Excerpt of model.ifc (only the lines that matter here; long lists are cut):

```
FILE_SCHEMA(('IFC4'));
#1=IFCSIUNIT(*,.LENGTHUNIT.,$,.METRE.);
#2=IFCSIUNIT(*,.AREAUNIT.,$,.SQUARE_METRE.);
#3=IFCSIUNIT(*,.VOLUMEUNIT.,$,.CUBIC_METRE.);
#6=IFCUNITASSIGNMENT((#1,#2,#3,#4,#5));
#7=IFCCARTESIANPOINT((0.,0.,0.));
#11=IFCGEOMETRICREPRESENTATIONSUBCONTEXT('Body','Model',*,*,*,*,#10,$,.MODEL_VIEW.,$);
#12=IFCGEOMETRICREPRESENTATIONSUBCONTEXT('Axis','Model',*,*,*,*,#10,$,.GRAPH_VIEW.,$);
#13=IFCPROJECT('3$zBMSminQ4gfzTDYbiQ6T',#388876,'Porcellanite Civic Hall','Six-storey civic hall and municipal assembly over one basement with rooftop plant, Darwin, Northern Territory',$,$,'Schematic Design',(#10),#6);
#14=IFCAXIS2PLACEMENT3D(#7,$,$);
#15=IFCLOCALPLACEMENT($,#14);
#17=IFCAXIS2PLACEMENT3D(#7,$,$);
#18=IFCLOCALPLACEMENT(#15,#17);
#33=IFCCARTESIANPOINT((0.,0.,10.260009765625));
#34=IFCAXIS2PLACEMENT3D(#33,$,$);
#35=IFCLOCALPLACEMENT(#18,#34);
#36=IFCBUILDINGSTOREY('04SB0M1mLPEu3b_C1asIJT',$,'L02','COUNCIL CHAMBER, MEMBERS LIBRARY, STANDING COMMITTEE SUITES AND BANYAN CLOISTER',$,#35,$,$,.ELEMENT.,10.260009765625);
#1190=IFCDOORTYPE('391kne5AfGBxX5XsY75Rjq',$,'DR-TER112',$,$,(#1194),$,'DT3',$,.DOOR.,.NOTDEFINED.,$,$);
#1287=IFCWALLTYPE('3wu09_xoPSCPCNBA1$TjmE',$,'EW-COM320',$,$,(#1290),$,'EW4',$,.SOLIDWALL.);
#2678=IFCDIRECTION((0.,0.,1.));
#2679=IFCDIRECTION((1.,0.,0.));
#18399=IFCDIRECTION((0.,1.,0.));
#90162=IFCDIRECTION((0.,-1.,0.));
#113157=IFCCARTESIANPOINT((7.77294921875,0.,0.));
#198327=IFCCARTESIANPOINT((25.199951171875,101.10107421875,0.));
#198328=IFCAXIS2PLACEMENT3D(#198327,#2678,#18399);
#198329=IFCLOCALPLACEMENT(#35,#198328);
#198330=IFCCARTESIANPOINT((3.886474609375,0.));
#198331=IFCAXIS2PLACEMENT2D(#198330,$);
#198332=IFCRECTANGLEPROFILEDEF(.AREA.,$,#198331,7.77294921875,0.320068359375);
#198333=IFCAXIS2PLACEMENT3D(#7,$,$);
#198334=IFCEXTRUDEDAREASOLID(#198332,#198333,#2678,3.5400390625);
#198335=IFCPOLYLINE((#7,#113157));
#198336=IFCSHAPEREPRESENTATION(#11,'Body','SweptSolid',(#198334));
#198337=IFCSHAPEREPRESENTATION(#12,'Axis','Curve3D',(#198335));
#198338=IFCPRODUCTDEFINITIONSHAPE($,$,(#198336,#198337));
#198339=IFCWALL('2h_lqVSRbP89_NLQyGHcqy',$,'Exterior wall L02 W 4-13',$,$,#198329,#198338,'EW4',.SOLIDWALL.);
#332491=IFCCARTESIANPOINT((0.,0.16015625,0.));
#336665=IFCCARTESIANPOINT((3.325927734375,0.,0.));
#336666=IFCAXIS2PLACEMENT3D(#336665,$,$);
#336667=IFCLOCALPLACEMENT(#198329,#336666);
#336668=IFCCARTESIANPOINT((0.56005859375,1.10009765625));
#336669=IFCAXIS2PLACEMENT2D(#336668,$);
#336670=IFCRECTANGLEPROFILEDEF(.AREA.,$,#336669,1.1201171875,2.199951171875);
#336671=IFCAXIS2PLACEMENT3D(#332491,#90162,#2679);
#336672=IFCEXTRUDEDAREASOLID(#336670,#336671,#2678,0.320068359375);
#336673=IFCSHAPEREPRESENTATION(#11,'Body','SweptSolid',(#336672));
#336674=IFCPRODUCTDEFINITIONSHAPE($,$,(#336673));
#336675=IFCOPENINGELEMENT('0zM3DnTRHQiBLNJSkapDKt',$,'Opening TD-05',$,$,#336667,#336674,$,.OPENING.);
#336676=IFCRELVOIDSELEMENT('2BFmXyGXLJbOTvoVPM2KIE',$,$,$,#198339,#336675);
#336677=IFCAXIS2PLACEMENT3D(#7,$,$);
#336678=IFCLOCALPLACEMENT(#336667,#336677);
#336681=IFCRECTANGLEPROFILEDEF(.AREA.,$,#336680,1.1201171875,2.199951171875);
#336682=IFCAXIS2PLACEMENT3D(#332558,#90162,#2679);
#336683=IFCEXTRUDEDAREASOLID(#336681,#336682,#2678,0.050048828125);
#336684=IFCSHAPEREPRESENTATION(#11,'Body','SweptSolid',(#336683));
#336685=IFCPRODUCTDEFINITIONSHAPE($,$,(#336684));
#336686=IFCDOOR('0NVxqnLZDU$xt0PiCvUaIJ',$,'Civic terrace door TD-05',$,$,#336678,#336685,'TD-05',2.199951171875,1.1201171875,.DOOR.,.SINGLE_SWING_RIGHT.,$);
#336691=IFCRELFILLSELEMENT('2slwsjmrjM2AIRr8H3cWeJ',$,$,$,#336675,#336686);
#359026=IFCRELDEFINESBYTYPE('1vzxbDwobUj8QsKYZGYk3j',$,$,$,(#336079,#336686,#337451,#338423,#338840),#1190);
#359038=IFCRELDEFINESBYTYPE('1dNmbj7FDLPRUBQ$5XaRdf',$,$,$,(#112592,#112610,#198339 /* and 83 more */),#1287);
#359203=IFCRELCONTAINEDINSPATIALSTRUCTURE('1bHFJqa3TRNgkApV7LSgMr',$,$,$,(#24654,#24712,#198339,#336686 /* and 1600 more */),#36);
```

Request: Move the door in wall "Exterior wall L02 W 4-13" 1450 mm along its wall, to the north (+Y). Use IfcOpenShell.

```python
import ifcopenshell
import ifcopenshell.api.geometry
import ifcopenshell.util.placement
import ifcopenshell.util.unit

model = ifcopenshell.open("model.ifc")
unit_scale = ifcopenshell.util.unit.calculate_unit_scale(model)

door = model.by_id(336686)
opening = door.FillsVoids[0].RelatingOpeningElement
wall = opening.VoidsElements[0].RelatingBuildingElement

wall_matrix = ifcopenshell.util.placement.get_local_placement(wall.ObjectPlacement)
shift = wall_matrix[:3, 0] * 1.45 / unit_scale
before = ifcopenshell.util.placement.get_local_placement(door.ObjectPlacement)[:3, 3].copy()

# The door is placed relative to its opening, so it follows when the opening moves.
matrix = ifcopenshell.util.placement.get_local_placement(opening.ObjectPlacement)
matrix[:3, 3] += shift
ifcopenshell.api.geometry.edit_object_placement(
    model, product=opening, matrix=matrix, is_si=False, should_transform_children=True
)

after = ifcopenshell.util.placement.get_local_placement(door.ObjectPlacement)[:3, 3]
print("door moved by", (after - before).round(3) + 0.0)

model.write("model_v2.ifc")
```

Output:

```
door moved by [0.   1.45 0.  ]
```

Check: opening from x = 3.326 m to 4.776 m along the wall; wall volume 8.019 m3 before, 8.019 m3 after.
